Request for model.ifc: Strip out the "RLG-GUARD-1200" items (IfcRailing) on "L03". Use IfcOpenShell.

First a look at what the model holds.

```python
import ifcopenshell
import ifcopenshell.util.element

model = ifcopenshell.open("model.ifc")
print(model.schema)
storey = next(s for s in model.by_type("IfcBuildingStorey") if s.Name == "L03")
railings = [e for e in ifcopenshell.util.element.get_decomposition(storey) if e.is_a("IfcRailing")]
seen = {}
for e in railings:
    element_type = ifcopenshell.util.element.get_type(e)
    name = element_type.Name if element_type not in (None, e) else None
    seen[name] = seen.get(name, 0) + 1
for name, count in sorted(seen.items(), key=str):
    print(count, "x", name)
```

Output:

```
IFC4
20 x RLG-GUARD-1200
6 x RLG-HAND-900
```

```python
import ifcopenshell
import ifcopenshell.api.root
import ifcopenshell.util.element

model = ifcopenshell.open("model.ifc")

storey = next(s for s in model.by_type("IfcBuildingStorey") if s.Name == "L03")
railings = [e for e in ifcopenshell.util.element.get_decomposition(storey) if e.is_a("IfcRailing")]
targets = [e for e in railings if (t := ifcopenshell.util.element.get_type(e)) not in (None, e) and t.Name == "RLG-GUARD-1200"]

for e in targets:
    ifcopenshell.api.root.remove_product(model, product=e)
print(len(targets), "removed")

model.write("model_rev.ifc")
```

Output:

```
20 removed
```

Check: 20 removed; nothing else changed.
